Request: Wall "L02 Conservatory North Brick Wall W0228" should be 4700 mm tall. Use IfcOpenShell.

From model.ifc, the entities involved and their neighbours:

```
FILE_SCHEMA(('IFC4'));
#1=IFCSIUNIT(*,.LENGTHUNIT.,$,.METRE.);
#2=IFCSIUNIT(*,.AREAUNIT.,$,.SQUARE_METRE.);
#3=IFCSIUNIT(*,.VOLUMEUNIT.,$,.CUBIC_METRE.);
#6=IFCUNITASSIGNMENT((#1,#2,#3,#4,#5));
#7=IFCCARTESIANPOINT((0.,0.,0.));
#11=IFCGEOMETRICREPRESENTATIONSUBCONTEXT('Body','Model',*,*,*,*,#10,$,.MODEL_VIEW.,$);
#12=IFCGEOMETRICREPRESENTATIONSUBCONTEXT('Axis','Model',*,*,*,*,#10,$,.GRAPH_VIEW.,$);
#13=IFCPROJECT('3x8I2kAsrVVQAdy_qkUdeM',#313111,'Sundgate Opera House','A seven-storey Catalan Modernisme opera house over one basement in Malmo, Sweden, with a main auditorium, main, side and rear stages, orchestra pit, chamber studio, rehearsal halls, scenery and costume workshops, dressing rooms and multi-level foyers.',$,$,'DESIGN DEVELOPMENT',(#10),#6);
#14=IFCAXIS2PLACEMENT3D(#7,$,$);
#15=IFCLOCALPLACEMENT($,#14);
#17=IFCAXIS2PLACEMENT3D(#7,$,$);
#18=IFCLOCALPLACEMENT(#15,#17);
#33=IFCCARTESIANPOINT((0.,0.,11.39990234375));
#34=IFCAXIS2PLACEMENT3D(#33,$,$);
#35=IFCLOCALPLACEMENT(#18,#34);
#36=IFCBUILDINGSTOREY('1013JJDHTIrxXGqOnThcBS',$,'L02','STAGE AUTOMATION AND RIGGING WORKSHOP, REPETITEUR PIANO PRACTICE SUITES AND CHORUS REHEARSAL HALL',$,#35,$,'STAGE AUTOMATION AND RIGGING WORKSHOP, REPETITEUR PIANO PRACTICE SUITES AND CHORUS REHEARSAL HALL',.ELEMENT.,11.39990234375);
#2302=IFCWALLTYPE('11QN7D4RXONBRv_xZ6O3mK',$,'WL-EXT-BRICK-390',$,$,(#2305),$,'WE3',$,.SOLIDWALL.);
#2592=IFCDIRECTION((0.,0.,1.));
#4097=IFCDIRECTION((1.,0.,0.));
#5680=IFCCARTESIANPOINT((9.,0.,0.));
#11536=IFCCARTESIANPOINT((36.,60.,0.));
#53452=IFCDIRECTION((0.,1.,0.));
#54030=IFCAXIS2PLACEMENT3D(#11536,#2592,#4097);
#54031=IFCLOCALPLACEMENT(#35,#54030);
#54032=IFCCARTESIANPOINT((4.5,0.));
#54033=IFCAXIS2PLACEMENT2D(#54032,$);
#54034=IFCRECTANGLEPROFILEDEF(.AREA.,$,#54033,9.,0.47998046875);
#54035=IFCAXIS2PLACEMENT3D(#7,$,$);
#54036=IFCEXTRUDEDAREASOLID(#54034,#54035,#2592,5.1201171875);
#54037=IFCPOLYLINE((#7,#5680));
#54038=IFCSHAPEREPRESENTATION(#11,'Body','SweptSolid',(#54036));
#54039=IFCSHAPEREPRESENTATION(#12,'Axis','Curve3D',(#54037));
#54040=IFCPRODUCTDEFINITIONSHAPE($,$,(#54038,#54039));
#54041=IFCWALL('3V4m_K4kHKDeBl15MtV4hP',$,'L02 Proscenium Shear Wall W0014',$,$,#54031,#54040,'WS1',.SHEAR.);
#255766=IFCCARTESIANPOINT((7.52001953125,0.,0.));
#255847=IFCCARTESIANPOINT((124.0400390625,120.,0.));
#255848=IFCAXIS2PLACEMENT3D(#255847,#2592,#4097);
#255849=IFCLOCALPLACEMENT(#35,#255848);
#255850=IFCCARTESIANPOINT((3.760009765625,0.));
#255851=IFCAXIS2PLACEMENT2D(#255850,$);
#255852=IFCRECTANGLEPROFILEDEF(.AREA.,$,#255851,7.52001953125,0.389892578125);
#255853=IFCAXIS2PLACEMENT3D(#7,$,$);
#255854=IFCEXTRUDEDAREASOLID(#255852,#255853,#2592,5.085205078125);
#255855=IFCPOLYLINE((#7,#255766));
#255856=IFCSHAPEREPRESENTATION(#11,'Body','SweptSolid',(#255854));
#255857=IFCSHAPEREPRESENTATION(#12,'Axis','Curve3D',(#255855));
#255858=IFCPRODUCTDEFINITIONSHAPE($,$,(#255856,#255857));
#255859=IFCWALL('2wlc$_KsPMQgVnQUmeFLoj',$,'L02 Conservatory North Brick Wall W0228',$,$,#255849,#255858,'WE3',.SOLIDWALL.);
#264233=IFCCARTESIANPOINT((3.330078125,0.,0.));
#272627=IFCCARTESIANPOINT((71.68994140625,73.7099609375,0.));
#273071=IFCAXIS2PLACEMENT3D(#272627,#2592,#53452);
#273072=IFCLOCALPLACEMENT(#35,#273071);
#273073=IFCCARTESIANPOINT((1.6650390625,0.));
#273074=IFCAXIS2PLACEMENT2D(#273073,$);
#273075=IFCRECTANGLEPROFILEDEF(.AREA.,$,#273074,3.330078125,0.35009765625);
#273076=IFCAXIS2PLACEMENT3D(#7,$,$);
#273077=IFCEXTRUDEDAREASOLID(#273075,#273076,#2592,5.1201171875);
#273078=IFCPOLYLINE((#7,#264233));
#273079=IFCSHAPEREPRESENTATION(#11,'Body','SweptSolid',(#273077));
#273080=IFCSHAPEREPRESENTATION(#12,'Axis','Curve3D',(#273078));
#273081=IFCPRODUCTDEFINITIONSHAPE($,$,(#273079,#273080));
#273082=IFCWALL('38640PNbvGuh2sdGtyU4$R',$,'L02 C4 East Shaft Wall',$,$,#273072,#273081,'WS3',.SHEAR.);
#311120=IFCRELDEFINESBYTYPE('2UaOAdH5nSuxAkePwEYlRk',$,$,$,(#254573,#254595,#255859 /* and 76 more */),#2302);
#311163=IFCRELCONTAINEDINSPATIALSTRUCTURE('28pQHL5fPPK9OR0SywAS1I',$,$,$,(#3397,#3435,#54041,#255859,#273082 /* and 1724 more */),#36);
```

```python
import ifcopenshell
import ifcopenshell.geom
import ifcopenshell.util.representation
import ifcopenshell.util.shape
import ifcopenshell.util.unit

model = ifcopenshell.open("model.ifc")
unit_scale = ifcopenshell.util.unit.calculate_unit_scale(model)
settings = ifcopenshell.geom.settings()


def volume(element):
    """Net volume in cubic metres, openings subtracted."""
    shape = ifcopenshell.geom.create_shape(settings, element)
    return ifcopenshell.util.shape.get_volume(shape.geometry)


wall = model.by_guid("2wlc$_KsPMQgVnQUmeFLoj")
before = volume(wall)

body = ifcopenshell.util.representation.get_representation(wall, "Model", "Body")
solid = body.Items[0]
old_height = solid.Depth
solid.Depth = 4.7 / unit_scale
after = volume(wall)

print(f"height {old_height:g} -> {solid.Depth:g}, volume {before:.3f} -> {after:.3f} m3")

model.write("model_updated.ifc")
```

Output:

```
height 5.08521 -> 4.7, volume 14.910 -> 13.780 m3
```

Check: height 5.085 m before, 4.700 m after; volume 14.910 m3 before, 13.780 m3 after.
